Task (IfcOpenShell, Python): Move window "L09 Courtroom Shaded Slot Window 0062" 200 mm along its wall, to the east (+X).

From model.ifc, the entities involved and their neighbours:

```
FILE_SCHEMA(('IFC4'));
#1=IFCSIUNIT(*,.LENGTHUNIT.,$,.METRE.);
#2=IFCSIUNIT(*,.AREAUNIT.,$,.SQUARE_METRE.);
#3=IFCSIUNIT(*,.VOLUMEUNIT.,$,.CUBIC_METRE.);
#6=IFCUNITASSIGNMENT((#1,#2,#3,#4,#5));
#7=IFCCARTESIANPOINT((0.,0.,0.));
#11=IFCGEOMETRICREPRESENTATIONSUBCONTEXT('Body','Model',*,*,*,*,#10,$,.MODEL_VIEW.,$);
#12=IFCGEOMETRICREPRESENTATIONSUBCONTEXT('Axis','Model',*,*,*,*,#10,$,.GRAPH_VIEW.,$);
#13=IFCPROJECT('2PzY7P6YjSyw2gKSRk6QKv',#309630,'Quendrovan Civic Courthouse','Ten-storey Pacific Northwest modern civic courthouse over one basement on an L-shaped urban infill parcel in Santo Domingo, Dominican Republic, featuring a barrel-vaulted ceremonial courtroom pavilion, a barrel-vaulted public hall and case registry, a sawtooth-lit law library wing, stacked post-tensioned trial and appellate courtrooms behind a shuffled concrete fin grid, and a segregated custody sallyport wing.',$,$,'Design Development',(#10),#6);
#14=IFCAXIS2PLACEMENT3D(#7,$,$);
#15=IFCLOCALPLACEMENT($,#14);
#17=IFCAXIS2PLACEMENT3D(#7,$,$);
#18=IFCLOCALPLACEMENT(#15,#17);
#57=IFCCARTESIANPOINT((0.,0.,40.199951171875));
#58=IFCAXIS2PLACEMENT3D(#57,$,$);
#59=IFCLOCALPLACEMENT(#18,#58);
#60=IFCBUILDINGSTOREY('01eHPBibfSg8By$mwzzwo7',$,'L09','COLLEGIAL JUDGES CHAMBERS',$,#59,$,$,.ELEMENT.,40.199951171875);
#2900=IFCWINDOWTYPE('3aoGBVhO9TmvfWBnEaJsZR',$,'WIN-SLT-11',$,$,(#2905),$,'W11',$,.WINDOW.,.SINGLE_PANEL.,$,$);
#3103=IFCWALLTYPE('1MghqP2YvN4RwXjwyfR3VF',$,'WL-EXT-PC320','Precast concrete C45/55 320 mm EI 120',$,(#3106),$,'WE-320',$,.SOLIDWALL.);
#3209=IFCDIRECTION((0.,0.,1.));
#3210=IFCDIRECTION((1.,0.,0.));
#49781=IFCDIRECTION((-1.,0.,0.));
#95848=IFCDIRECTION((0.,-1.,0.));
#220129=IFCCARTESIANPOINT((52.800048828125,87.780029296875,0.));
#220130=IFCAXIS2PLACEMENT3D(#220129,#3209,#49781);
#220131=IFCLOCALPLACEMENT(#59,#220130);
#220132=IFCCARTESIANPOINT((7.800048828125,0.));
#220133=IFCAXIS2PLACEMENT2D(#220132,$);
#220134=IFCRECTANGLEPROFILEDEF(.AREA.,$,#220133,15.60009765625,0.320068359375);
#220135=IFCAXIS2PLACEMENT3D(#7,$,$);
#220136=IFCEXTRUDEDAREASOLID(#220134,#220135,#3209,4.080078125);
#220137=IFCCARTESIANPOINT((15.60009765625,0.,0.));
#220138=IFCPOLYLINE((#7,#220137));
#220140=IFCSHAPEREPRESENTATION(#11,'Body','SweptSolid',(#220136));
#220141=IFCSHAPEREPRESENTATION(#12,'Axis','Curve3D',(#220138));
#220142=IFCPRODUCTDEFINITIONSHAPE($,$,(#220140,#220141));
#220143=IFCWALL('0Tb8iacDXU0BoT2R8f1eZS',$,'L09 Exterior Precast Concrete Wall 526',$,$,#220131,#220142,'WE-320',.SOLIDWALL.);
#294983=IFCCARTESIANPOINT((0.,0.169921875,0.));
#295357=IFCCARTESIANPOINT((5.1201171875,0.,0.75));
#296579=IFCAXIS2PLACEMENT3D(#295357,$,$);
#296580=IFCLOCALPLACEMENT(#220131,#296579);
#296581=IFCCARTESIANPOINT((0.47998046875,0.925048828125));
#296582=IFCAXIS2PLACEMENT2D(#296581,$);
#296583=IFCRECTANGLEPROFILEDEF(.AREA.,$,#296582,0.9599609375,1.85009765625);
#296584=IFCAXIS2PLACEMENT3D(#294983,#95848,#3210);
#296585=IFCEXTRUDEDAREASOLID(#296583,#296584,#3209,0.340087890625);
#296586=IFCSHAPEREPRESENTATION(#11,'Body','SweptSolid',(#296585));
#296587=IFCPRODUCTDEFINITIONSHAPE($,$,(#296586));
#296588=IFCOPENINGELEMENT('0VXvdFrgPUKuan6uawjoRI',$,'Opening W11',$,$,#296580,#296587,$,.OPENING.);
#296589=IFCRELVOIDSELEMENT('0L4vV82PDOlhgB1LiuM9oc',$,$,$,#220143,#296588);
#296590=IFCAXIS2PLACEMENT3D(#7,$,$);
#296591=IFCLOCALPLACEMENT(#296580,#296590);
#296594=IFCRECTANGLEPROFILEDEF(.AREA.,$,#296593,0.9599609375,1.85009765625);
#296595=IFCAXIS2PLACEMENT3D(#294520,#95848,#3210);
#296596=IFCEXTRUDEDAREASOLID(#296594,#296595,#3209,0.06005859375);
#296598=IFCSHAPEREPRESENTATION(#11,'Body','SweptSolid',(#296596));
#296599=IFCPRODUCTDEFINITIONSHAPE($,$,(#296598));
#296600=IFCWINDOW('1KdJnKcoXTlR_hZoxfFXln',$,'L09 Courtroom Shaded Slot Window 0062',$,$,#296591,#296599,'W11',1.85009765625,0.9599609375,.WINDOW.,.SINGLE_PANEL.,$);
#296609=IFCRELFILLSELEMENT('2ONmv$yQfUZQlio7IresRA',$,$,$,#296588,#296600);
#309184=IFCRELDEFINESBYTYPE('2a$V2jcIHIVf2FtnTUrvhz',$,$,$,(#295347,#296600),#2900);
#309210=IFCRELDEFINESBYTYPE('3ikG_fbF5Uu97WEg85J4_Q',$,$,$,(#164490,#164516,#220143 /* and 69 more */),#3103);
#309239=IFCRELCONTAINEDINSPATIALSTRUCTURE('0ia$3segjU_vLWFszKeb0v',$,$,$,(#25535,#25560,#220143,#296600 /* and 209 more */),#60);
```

```python
import ifcopenshell
import ifcopenshell.api.geometry
import ifcopenshell.util.placement

model = ifcopenshell.open("model.ifc")

window = model.by_guid("1KdJnKcoXTlR_hZoxfFXln")
opening = window.FillsVoids[0].RelatingOpeningElement
wall = opening.VoidsElements[0].RelatingBuildingElement

wall_matrix = ifcopenshell.util.placement.get_local_placement(wall.ObjectPlacement)
shift = wall_matrix[:3, 0] * -0.2
before = ifcopenshell.util.placement.get_local_placement(window.ObjectPlacement)[:3, 3].copy()

# The window is placed relative to its opening, so it follows when the opening moves.
matrix = ifcopenshell.util.placement.get_local_placement(opening.ObjectPlacement)
matrix[:3, 3] += shift
ifcopenshell.api.geometry.edit_object_placement(
    model, product=opening, matrix=matrix, is_si=False, should_transform_children=True
)

after = ifcopenshell.util.placement.get_local_placement(window.ObjectPlacement)[:3, 3]
print("window moved by", (after - before).round(3) + 0.0)

model.write("model_edited.ifc")
```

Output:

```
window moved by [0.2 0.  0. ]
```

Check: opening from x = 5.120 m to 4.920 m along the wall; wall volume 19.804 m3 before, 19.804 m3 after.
